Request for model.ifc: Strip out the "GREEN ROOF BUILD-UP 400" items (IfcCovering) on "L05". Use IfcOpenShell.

First a look at what the model holds.

```python
import ifcopenshell
import ifcopenshell.util.element

model = ifcopenshell.open("model.ifc")
print(model.schema)
storey = next(s for s in model.by_type("IfcBuildingStorey") if s.Name == "L05")
coverings = [e for e in ifcopenshell.util.element.get_decomposition(storey) if e.is_a("IfcCovering")]
seen = {}
for e in coverings:
    element_type = ifcopenshell.util.element.get_type(e)
    name = element_type.Name if element_type not in (None, e) else None
    seen[name] = seen.get(name, 0) + 1
for name, count in sorted(seen.items(), key=str):
    print(count, "x", name)
```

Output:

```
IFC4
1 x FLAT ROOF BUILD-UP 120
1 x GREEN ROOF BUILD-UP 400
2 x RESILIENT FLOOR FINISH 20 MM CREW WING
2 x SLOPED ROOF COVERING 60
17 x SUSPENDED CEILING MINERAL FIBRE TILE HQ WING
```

```python
import ifcopenshell
import ifcopenshell.api.root
import ifcopenshell.util.element

model = ifcopenshell.open("model.ifc")

storey = next(s for s in model.by_type("IfcBuildingStorey") if s.Name == "L05")
coverings = [e for e in ifcopenshell.util.element.get_decomposition(storey) if e.is_a("IfcCovering")]
targets = [e for e in coverings if (t := ifcopenshell.util.element.get_type(e)) not in (None, e) and t.Name == "GREEN ROOF BUILD-UP 400"]

for e in targets:
    ifcopenshell.api.root.remove_product(model, product=e)
print(len(targets), "removed")

model.write("model_updated.ifc")
```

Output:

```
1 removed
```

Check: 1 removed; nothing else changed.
